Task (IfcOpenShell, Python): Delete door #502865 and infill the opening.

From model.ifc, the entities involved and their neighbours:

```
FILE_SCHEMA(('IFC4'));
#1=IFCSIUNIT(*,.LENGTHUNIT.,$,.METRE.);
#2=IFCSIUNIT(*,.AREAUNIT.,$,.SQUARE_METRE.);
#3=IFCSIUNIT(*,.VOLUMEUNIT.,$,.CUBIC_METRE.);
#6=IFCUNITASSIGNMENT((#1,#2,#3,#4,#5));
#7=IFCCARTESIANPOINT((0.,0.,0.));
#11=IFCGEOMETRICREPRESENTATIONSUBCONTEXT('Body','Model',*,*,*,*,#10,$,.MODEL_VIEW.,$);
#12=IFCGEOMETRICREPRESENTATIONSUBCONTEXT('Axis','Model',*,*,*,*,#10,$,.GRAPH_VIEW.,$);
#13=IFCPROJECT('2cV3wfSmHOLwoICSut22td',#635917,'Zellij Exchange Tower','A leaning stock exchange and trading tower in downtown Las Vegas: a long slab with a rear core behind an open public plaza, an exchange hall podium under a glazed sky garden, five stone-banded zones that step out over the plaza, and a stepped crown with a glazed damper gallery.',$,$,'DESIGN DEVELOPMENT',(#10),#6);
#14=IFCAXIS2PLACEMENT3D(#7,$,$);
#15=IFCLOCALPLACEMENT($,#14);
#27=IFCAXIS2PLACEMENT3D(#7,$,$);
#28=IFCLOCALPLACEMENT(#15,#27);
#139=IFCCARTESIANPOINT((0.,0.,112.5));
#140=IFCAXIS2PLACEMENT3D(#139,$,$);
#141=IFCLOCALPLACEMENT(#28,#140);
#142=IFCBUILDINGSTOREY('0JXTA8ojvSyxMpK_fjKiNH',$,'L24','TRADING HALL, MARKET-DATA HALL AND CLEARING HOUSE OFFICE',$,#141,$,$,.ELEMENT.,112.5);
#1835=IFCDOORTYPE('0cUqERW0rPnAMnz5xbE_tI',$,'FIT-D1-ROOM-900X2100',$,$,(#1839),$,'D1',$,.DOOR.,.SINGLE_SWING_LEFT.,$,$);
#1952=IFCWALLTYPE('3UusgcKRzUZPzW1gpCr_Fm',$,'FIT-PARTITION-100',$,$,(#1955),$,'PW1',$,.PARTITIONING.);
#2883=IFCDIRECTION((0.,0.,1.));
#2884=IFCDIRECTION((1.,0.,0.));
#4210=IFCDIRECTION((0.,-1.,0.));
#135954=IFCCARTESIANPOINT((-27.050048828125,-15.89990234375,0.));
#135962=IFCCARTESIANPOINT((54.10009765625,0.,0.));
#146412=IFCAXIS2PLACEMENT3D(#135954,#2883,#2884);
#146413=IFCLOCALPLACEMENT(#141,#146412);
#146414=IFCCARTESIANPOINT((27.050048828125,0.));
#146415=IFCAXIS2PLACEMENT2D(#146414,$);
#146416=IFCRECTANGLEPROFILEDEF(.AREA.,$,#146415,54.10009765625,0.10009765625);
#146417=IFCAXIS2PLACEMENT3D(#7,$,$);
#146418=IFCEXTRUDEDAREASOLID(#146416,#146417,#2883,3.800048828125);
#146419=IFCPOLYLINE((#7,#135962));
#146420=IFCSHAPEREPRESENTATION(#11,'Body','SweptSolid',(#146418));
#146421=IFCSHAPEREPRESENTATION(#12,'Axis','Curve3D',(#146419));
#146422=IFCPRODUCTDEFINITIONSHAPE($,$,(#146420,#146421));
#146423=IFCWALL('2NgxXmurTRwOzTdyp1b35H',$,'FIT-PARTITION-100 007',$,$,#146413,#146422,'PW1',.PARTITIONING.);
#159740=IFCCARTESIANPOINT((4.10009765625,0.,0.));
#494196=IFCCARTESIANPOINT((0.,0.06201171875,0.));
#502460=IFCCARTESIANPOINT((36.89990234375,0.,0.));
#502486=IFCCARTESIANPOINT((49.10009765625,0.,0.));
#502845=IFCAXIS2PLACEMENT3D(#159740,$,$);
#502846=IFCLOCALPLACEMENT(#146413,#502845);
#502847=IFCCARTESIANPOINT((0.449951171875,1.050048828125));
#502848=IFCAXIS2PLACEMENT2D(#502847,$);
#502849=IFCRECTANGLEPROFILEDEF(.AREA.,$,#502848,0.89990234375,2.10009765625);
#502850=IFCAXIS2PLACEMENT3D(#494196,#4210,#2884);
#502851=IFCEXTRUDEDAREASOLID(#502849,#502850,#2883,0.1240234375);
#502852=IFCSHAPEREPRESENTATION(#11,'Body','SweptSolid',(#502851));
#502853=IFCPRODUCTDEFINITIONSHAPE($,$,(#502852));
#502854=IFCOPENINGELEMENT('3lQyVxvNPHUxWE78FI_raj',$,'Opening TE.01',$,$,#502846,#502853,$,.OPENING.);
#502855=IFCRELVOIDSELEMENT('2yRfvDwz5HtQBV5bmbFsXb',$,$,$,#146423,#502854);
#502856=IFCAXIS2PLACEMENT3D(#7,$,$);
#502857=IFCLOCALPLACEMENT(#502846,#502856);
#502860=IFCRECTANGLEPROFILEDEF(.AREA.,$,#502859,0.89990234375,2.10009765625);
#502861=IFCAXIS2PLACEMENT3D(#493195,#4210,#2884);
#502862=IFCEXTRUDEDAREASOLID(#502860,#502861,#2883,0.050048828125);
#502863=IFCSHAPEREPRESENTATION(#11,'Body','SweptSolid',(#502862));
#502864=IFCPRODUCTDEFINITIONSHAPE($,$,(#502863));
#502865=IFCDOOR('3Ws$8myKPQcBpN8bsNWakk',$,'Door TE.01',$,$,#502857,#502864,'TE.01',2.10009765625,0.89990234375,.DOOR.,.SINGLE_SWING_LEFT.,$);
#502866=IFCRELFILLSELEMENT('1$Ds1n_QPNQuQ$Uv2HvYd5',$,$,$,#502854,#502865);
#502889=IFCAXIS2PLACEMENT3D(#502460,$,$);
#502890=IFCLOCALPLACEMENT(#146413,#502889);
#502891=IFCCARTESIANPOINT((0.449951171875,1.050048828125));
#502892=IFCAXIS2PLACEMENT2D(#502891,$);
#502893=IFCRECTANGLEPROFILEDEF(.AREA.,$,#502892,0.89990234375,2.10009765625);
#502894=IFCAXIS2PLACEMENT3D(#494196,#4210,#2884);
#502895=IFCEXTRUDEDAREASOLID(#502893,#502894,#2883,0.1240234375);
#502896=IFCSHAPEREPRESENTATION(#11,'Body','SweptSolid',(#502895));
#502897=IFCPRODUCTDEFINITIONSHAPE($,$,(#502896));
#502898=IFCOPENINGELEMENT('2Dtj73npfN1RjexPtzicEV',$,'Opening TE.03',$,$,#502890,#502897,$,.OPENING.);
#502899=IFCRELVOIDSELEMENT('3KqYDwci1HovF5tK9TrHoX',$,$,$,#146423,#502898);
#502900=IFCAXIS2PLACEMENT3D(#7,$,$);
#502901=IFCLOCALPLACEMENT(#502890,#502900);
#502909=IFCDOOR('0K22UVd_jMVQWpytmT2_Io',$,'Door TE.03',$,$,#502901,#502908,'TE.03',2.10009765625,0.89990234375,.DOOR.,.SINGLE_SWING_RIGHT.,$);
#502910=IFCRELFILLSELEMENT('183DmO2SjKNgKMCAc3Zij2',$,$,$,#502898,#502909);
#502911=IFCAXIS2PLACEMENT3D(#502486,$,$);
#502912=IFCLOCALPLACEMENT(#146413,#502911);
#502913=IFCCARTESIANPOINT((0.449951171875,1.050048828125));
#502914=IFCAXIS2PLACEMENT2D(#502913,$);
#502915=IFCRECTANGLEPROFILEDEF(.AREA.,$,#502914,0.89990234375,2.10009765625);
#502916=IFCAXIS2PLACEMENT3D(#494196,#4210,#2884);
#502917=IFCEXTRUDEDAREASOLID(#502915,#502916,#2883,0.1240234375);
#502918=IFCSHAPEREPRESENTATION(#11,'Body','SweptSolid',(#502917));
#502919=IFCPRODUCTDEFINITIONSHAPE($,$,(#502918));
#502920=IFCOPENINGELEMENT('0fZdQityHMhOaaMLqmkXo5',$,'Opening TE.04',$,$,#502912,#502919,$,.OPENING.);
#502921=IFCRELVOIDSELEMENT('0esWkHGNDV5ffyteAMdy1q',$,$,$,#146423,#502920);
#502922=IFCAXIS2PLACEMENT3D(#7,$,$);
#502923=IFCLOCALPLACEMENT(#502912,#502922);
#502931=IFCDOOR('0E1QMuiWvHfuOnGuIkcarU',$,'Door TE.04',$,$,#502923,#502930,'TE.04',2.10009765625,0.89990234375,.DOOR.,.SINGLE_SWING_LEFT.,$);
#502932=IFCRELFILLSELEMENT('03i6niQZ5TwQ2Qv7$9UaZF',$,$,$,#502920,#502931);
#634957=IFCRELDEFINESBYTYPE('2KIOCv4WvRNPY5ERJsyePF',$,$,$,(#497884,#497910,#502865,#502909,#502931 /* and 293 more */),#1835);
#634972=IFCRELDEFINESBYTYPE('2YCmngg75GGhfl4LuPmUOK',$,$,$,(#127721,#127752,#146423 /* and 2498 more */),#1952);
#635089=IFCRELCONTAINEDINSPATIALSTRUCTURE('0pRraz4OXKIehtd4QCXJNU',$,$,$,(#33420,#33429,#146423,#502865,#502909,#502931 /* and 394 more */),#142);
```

```python
import ifcopenshell
import ifcopenshell.api.feature
import ifcopenshell.api.root
import ifcopenshell.geom
import ifcopenshell.util.shape

model = ifcopenshell.open("model.ifc")
settings = ifcopenshell.geom.settings()


def volume(element):
    """Net volume in cubic metres, openings subtracted."""
    shape = ifcopenshell.geom.create_shape(settings, element)
    return ifcopenshell.util.shape.get_volume(shape.geometry)


door = model.by_guid("3Ws$8myKPQcBpN8bsNWakk")
opening = door.FillsVoids[0].RelatingOpeningElement
wall = opening.VoidsElements[0].RelatingBuildingElement
before = volume(wall)

ifcopenshell.api.root.remove_product(model, product=door)
ifcopenshell.api.feature.remove_feature(model, feature=opening)

after = volume(wall)

print(f"wall volume {before:.3f} -> {after:.3f} m3")

model.write("model_edited.ifc")
```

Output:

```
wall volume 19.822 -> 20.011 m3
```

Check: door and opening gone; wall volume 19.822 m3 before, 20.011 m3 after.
